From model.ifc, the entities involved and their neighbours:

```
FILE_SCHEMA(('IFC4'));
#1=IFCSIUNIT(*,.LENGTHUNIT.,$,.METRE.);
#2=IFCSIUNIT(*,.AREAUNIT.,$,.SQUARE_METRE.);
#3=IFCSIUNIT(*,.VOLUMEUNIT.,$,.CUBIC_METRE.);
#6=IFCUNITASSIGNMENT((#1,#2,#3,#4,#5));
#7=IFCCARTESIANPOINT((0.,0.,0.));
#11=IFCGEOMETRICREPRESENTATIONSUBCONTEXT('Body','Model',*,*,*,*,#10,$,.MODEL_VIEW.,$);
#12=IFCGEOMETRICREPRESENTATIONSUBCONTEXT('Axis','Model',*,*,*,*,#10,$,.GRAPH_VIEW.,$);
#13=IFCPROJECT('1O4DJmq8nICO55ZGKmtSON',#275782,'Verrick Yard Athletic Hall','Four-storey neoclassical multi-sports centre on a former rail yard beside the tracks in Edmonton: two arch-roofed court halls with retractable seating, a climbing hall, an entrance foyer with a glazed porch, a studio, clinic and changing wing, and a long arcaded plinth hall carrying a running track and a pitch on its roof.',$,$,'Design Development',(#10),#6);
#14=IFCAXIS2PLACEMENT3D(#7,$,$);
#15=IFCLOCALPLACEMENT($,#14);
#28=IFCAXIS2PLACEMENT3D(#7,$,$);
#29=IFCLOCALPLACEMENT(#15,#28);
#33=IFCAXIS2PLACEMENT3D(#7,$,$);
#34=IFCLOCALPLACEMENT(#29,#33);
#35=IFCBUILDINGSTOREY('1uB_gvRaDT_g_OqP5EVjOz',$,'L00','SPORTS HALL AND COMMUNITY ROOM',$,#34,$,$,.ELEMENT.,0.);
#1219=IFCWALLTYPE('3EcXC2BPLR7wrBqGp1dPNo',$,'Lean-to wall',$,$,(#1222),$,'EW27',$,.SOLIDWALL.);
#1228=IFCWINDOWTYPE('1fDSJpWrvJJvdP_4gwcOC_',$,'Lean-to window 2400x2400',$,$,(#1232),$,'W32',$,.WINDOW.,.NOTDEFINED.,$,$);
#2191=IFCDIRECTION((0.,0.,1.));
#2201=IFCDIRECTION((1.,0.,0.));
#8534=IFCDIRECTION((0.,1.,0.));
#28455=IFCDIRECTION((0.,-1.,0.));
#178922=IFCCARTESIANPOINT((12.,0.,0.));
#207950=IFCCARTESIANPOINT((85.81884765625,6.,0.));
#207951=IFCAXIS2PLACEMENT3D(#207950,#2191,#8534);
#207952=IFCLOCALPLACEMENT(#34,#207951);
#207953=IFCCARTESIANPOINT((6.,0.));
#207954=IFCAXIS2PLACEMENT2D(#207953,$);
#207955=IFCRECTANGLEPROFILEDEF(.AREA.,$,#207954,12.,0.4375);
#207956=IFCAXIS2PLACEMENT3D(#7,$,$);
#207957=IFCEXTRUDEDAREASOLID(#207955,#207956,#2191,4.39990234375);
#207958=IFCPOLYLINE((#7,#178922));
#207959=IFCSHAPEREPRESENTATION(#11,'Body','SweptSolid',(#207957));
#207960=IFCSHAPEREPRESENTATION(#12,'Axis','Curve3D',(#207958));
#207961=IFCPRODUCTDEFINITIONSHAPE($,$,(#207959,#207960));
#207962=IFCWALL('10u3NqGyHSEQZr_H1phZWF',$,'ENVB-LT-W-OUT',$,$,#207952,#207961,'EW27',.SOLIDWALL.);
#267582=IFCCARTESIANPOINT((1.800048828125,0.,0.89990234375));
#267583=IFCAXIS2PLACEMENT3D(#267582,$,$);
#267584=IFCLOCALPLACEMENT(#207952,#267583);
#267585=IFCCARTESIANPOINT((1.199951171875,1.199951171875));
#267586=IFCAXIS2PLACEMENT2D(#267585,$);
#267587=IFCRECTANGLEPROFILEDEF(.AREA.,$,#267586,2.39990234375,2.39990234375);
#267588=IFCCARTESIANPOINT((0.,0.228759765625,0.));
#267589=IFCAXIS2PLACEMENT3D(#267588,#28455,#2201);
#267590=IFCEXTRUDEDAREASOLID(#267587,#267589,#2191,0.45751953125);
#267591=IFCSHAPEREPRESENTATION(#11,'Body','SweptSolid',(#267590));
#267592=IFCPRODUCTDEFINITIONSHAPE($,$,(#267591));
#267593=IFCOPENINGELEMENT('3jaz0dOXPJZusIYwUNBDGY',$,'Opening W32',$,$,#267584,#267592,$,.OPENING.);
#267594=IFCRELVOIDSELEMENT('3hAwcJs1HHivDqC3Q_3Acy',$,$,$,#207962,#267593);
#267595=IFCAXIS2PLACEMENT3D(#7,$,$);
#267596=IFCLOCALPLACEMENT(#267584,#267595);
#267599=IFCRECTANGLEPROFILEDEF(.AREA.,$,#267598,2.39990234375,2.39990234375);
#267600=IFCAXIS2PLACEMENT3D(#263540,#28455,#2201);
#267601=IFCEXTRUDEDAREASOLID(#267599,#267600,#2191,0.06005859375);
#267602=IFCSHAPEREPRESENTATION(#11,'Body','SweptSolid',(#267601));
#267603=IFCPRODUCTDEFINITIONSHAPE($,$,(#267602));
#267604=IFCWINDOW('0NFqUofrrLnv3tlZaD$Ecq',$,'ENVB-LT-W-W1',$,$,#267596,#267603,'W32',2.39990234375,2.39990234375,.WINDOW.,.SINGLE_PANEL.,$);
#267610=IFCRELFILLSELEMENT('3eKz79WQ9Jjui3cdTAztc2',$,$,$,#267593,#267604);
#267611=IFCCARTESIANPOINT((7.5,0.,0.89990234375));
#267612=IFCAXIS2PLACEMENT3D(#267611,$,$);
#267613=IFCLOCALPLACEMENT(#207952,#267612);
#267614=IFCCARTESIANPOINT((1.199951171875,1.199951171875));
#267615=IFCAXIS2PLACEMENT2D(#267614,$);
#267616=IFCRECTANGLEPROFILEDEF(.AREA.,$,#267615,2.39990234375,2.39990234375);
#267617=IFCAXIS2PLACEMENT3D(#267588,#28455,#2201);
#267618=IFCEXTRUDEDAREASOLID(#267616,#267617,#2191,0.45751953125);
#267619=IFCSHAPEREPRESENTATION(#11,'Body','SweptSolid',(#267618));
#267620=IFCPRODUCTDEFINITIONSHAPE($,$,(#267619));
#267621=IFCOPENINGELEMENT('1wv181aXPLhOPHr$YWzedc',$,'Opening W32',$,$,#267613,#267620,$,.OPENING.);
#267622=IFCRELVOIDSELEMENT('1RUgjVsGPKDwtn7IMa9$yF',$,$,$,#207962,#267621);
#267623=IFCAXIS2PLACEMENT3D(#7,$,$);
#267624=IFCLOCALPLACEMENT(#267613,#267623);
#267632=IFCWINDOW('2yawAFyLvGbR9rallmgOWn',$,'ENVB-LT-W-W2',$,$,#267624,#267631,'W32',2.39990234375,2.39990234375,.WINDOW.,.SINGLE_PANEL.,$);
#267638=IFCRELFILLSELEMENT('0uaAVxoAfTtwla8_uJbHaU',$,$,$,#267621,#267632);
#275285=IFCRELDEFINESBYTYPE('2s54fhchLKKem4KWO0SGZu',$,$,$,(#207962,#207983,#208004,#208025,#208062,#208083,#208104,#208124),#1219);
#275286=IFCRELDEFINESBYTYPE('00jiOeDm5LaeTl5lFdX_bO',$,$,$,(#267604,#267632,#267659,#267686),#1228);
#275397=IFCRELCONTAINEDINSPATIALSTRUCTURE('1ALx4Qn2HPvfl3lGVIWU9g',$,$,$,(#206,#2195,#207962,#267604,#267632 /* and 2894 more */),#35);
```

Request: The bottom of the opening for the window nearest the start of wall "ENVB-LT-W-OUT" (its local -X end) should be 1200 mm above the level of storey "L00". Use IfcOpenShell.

```python
import numpy as np
import ifcopenshell
import ifcopenshell.api.geometry
import ifcopenshell.geom
import ifcopenshell.util.element
import ifcopenshell.util.placement
import ifcopenshell.util.shape
import ifcopenshell.util.unit

model = ifcopenshell.open("model.ifc")
unit_scale = ifcopenshell.util.unit.calculate_unit_scale(model)

window = model.by_guid("0NFqUofrrLnv3tlZaD$Ecq")
opening = window.FillsVoids[0].RelatingOpeningElement
storey = ifcopenshell.util.element.get_container(window, ifc_class="IfcBuildingStorey")
level = ifcopenshell.util.placement.get_local_placement(storey.ObjectPlacement)[2, 3]

# The opening's origin need not be at the sill, so measure its lowest point.
shape = ifcopenshell.geom.create_shape(ifcopenshell.geom.settings(), opening)
bottom = ifcopenshell.util.shape.get_shape_bottom_elevation(shape, shape.geometry) / unit_scale
dz = level + 1.2 / unit_scale - bottom

shift = np.array([0.0, 0.0, dz])
# The window is placed relative to its opening, so it follows when the opening moves.
matrix = ifcopenshell.util.placement.get_local_placement(opening.ObjectPlacement)
matrix[:3, 3] += shift
ifcopenshell.api.geometry.edit_object_placement(
    model, product=opening, matrix=matrix, is_si=False, should_transform_children=True
)

print(f"moved by {dz * unit_scale:+.3f} m")

model.write("model_updated.ifc")
```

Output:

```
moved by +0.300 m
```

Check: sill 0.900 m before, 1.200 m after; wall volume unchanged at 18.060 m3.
